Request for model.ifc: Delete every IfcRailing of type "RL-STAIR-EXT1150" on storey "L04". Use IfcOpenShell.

First a look at what the model holds.

```python
import ifcopenshell
import ifcopenshell.util.element

model = ifcopenshell.open("model.ifc")
print(model.schema)
storey = next(s for s in model.by_type("IfcBuildingStorey") if s.Name == "L04")
railings = [e for e in ifcopenshell.util.element.get_decomposition(storey) if e.is_a("IfcRailing")]
seen = {}
for e in railings:
    element_type = ifcopenshell.util.element.get_type(e)
    name = element_type.Name if element_type not in (None, e) else None
    seen[name] = seen.get(name, 0) + 1
for name, count in sorted(seen.items(), key=str):
    print(count, "x", name)
```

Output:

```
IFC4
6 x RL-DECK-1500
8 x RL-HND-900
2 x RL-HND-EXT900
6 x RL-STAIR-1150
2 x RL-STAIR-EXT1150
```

```python
import ifcopenshell
import ifcopenshell.api.root
import ifcopenshell.util.element

model = ifcopenshell.open("model.ifc")

storey = next(s for s in model.by_type("IfcBuildingStorey") if s.Name == "L04")
railings = [e for e in ifcopenshell.util.element.get_decomposition(storey) if e.is_a("IfcRailing")]
targets = [e for e in railings if (t := ifcopenshell.util.element.get_type(e)) not in (None, e) and t.Name == "RL-STAIR-EXT1150"]

for e in targets:
    ifcopenshell.api.root.remove_product(model, product=e)
print(len(targets), "removed")

model.write("model_updated.ifc")
```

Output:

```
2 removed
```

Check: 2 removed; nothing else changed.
